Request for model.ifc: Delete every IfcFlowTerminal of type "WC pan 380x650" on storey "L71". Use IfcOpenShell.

First a look at what the model holds.

```python
import ifcopenshell
import ifcopenshell.util.element

model = ifcopenshell.open("model.ifc")
print(model.schema)
storey = next(s for s in model.by_type("IfcBuildingStorey") if s.Name == "L71")
terminals = [e for e in ifcopenshell.util.element.get_decomposition(storey) if e.is_a("IfcFlowTerminal")]
seen = {}
for e in terminals:
    element_type = ifcopenshell.util.element.get_type(e)
    name = element_type.Name if element_type not in (None, e) else None
    seen[name] = seen.get(name, 0) + 1
for name, count in sorted(seen.items(), key=str):
    print(count, "x", name)
```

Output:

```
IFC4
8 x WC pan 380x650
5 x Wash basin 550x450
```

```python
import ifcopenshell
import ifcopenshell.api.root
import ifcopenshell.util.element

model = ifcopenshell.open("model.ifc")

storey = next(s for s in model.by_type("IfcBuildingStorey") if s.Name == "L71")
terminals = [e for e in ifcopenshell.util.element.get_decomposition(storey) if e.is_a("IfcFlowTerminal")]
targets = [e for e in terminals if (t := ifcopenshell.util.element.get_type(e)) not in (None, e) and t.Name == "WC pan 380x650"]

for e in targets:
    ifcopenshell.api.root.remove_product(model, product=e)
print(len(targets), "removed")

model.write("model-out.ifc")
```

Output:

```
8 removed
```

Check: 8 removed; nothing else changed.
